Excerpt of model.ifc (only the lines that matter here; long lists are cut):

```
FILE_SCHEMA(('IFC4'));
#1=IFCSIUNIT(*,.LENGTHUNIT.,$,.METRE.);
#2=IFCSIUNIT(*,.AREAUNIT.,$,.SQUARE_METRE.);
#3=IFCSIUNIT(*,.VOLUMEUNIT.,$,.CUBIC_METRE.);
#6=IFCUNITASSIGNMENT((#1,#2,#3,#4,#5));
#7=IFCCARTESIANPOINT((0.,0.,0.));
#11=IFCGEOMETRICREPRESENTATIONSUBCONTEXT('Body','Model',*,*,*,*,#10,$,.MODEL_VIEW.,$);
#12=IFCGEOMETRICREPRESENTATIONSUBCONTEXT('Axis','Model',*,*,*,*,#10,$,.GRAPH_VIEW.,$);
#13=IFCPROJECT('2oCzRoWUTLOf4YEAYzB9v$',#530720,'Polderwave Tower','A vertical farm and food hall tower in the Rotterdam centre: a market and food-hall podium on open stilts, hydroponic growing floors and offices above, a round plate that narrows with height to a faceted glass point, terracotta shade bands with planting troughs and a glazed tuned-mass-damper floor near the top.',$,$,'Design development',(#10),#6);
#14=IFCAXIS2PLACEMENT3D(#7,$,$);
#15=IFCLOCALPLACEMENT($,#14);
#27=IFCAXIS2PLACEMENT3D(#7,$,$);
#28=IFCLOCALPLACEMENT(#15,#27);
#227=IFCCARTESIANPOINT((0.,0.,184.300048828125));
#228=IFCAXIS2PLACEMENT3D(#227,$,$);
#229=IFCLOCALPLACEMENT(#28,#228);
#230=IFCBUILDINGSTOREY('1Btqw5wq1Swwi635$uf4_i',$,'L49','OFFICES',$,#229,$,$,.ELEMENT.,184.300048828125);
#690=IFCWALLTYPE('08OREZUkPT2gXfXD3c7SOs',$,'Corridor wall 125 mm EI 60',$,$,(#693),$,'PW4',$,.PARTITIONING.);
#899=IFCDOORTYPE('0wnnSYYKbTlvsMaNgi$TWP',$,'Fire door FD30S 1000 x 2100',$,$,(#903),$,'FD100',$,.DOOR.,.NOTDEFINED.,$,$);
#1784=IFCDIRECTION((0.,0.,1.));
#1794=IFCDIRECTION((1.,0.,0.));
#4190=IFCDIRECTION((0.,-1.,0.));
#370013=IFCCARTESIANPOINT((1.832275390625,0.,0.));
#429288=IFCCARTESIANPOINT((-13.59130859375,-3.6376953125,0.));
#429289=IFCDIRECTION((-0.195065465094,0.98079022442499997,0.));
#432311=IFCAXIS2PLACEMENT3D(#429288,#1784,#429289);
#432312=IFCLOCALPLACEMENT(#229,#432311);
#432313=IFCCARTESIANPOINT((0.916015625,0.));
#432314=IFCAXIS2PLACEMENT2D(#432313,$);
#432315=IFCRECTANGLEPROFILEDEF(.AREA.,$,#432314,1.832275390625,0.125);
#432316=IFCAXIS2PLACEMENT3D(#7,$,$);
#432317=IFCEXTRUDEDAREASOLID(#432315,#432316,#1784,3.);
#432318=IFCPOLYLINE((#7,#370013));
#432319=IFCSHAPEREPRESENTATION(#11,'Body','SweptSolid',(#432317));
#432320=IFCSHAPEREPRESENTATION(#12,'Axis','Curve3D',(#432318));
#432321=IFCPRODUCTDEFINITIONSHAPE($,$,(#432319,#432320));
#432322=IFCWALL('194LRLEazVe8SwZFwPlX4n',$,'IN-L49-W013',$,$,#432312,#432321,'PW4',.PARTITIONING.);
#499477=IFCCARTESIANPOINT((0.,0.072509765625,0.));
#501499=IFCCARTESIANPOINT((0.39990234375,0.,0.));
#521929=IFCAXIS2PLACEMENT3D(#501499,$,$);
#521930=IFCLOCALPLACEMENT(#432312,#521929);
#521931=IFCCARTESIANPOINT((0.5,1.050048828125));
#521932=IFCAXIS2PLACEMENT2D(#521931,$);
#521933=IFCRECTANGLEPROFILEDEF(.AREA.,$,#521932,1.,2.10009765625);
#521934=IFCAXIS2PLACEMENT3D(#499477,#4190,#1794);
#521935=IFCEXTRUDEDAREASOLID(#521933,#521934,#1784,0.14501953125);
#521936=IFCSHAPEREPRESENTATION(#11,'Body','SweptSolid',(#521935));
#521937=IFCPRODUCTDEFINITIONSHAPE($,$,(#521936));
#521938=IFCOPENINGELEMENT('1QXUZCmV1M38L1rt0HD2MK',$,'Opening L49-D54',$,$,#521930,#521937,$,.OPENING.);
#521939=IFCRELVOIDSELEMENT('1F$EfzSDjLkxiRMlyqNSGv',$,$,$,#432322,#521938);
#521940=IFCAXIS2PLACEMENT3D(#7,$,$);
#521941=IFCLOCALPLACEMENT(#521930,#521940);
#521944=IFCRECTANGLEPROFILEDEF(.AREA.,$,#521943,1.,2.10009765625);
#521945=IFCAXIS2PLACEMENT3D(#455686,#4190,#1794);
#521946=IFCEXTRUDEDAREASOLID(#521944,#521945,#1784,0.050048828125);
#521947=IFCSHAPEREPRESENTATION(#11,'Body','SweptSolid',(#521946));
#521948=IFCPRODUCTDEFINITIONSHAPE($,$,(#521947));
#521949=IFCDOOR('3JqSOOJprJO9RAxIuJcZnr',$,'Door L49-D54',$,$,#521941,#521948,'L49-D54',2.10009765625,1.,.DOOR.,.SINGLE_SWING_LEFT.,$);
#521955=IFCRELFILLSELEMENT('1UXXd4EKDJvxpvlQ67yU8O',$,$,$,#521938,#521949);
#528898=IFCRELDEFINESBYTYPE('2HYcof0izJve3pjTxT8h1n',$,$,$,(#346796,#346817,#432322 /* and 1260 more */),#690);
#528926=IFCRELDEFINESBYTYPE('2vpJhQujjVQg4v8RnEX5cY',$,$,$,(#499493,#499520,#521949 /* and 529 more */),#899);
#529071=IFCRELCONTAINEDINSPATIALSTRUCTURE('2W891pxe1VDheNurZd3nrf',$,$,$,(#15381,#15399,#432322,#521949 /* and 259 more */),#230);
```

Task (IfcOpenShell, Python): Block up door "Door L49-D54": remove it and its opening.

```python
import ifcopenshell
import ifcopenshell.api.feature
import ifcopenshell.api.root
import ifcopenshell.geom
import ifcopenshell.util.shape

model = ifcopenshell.open("model.ifc")
settings = ifcopenshell.geom.settings()


def volume(element):
    """Net volume in cubic metres, openings subtracted."""
    shape = ifcopenshell.geom.create_shape(settings, element)
    return ifcopenshell.util.shape.get_volume(shape.geometry)


door = model.by_guid("3JqSOOJprJO9RAxIuJcZnr")
opening = door.FillsVoids[0].RelatingOpeningElement
wall = opening.VoidsElements[0].RelatingBuildingElement
before = volume(wall)

ifcopenshell.api.root.remove_product(model, product=door)
ifcopenshell.api.feature.remove_feature(model, feature=opening)

after = volume(wall)

print(f"wall volume {before:.3f} -> {after:.3f} m3")

model.write("model_updated.ifc")
```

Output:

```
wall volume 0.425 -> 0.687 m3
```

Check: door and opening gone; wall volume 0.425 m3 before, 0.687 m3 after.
